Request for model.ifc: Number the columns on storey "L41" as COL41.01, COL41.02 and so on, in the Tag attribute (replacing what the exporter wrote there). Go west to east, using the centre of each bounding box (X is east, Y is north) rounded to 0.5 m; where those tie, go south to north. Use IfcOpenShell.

First a look at what the model holds.

```python
import ifcopenshell
import ifcopenshell.util.element
import ifcopenshell.util.placement

model = ifcopenshell.open("model.ifc")
print(model.schema)
storey = next(s for s in model.by_type("IfcBuildingStorey") if s.Name == "L41")
columns = [e for e in ifcopenshell.util.element.get_decomposition(storey) if e.is_a("IfcColumn")]
for e in sorted(columns, key=lambda e: e.id()):
    origin = ifcopenshell.util.placement.get_local_placement(e.ObjectPlacement)[:3, 3]
    print(e.id(), e.Tag, e.Name, origin.round(2) + 0.0, sep=" | ")
```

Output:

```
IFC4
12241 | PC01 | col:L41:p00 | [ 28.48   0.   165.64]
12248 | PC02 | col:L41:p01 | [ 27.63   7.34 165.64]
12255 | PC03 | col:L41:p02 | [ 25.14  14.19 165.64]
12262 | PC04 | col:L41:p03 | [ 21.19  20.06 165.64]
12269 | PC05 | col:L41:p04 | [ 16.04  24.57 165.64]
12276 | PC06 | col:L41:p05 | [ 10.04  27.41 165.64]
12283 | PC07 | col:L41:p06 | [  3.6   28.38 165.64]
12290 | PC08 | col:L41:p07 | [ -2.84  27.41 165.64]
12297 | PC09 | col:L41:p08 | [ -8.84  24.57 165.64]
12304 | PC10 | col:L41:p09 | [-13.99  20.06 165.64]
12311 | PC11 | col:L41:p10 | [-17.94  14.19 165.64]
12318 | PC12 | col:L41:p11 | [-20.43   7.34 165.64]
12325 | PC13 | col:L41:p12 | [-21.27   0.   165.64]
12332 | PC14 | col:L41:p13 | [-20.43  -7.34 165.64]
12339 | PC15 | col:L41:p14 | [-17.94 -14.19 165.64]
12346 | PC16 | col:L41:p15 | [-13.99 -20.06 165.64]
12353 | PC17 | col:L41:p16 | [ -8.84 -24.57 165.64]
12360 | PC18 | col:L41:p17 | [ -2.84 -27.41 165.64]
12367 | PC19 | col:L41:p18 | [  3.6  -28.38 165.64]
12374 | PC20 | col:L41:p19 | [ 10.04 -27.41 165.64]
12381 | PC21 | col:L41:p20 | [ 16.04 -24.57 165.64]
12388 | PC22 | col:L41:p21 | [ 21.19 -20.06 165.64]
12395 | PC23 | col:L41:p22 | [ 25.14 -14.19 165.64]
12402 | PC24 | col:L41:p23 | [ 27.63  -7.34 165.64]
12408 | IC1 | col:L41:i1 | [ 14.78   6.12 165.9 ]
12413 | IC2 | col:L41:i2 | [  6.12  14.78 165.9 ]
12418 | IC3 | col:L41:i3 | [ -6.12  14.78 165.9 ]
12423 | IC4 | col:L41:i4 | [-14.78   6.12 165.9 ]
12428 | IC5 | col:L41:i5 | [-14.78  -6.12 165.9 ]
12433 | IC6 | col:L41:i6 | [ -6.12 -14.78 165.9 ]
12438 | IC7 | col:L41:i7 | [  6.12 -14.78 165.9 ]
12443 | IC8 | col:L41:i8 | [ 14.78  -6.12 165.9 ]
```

```python
import ifcopenshell
import ifcopenshell.geom
import ifcopenshell.util.element
import ifcopenshell.util.shape

model = ifcopenshell.open("model.ifc")
settings = ifcopenshell.geom.settings()
settings.set("use-world-coords", True)


def centre(element):
    shape = ifcopenshell.geom.create_shape(settings, element)
    return ifcopenshell.util.shape.get_bbox_centroid(shape.geometry)


storey = next(s for s in model.by_type("IfcBuildingStorey") if s.Name == "L41")
columns = [e for e in ifcopenshell.util.element.get_decomposition(storey) if e.is_a("IfcColumn")]

# Insertion points can sit at a corner or the storey origin, so sort by the geometry (in metres).
centres = {e: centre(e) for e in columns}
columns.sort(key=lambda e: (round(centres[e][0] / 0.5), centres[e][1]))

for i, e in enumerate(columns, start=1):
    number = f"COL41.{i:02d}"
    e.Tag = number
    print(e.id(), number)

model.write("model_updated.ifc")
```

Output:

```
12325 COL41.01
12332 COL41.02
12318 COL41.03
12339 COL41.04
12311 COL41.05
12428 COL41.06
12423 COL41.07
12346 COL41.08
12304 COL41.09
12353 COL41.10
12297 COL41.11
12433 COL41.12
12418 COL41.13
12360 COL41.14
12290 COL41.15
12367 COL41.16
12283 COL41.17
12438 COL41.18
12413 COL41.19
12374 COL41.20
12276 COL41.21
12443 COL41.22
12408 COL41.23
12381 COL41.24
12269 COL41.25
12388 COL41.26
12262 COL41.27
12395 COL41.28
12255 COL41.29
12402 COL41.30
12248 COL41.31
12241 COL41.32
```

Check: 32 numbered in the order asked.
